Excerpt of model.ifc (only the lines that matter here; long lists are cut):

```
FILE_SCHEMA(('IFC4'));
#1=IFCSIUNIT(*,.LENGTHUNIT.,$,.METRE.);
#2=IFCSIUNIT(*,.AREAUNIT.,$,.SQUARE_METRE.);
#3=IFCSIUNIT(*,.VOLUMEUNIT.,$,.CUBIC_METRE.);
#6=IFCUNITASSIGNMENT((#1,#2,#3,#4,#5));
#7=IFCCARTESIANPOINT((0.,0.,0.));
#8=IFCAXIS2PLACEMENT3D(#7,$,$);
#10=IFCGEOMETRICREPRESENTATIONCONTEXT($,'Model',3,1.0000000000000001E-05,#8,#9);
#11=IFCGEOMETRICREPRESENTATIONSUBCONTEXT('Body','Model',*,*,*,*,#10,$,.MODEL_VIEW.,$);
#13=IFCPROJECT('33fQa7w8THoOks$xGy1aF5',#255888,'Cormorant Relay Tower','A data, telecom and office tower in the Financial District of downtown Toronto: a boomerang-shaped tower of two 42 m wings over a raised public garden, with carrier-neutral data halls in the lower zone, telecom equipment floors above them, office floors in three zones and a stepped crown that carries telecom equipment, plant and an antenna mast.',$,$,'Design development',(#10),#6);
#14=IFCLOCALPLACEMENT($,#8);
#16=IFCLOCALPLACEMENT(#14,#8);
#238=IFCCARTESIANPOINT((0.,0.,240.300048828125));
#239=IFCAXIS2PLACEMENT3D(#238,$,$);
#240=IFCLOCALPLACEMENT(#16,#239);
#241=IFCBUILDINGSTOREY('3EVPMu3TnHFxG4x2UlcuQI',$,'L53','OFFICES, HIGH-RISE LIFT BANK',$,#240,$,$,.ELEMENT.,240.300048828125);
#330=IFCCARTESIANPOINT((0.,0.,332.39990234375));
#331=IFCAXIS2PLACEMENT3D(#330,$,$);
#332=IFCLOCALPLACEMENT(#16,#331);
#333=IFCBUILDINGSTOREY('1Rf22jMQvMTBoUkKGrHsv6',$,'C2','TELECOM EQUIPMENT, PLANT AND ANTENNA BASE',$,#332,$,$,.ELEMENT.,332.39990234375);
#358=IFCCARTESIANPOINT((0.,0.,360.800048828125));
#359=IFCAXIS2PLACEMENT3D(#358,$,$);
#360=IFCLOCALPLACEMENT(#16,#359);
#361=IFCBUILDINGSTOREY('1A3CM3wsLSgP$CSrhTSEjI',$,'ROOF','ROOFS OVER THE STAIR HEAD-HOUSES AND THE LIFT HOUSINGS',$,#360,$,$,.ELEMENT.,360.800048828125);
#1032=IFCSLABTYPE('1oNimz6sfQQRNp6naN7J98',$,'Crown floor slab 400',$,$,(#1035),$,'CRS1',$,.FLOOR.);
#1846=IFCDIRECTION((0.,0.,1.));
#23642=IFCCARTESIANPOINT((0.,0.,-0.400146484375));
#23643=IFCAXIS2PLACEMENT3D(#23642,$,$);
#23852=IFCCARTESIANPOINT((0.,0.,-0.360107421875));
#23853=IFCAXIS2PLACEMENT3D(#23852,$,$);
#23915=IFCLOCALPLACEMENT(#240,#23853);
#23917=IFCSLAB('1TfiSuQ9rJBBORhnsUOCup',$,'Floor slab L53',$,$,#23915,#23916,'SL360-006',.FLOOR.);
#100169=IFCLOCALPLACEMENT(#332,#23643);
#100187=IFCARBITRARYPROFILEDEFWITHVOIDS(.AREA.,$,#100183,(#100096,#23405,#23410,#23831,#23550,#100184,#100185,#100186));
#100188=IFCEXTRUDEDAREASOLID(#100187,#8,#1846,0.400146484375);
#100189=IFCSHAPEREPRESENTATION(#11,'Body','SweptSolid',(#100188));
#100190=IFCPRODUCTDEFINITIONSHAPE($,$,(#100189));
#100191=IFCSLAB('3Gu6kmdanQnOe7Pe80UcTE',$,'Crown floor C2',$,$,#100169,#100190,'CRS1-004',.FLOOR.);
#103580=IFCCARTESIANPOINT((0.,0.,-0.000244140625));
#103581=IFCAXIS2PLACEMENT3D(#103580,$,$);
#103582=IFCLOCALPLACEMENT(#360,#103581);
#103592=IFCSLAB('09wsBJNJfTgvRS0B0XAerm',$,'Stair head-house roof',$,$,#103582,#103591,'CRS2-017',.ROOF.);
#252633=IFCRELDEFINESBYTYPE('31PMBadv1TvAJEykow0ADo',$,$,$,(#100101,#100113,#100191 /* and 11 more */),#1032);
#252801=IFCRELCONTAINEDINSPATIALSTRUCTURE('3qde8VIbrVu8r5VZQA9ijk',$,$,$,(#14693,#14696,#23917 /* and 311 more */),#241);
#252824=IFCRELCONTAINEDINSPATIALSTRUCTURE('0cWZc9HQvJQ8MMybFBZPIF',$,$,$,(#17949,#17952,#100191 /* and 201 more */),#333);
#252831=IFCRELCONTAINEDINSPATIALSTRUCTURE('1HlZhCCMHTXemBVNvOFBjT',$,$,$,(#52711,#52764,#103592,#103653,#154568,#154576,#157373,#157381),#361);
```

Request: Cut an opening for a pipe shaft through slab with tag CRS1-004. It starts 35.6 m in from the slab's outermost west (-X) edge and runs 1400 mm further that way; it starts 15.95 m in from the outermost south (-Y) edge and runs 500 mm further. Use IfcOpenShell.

```python
import numpy as np
import ifcopenshell
import ifcopenshell.api.feature
import ifcopenshell.api.geometry
import ifcopenshell.api.root
import ifcopenshell.geom
import ifcopenshell.util.placement
import ifcopenshell.util.representation
import ifcopenshell.util.shape
import ifcopenshell.util.unit

model = ifcopenshell.open("model.ifc")
unit_scale = ifcopenshell.util.unit.calculate_unit_scale(model)
settings = ifcopenshell.geom.settings()


def volume(element):
    """Net volume in cubic metres, openings subtracted."""
    shape = ifcopenshell.geom.create_shape(settings, element)
    return ifcopenshell.util.shape.get_volume(shape.geometry)


slab = model.by_id(100191)
before = volume(slab)

# Extent in the slab's own axes, in metres. The edges named are its -X and -Y sides.
slab_shape = ifcopenshell.geom.create_shape(settings, slab)
vertices = ifcopenshell.util.shape.get_vertices(slab_shape.geometry)
x_min, y_min, bottom = vertices.min(axis=0)
top = vertices[:, 2].max()

opening = ifcopenshell.api.root.create_entity(model, ifc_class="IfcOpeningElement", name="Pipe shaft opening", predefined_type="OPENING")
context = ifcopenshell.util.representation.get_context(model, "Model", "Body", "MODEL_VIEW")
width, depth = 1.4, 0.5
outline = [(0.0, 0.0), (width, 0.0), (width, depth), (0.0, depth), (0.0, 0.0)]
# Overshoot both faces by 50 mm so the cut is clean.
shape = ifcopenshell.api.geometry.add_slab_representation(
    model, context=context, depth=top - bottom + 0.1, polyline=outline
)
ifcopenshell.api.geometry.assign_representation(model, product=opening, representation=shape)

matrix = ifcopenshell.util.placement.get_local_placement(slab.ObjectPlacement)
matrix[:, 3] = matrix @ np.append(np.array([x_min + 35.6, y_min + 15.95, bottom - 0.05]) / unit_scale, 1.0)
ifcopenshell.api.geometry.edit_object_placement(model, product=opening, matrix=matrix, is_si=False)
ifcopenshell.api.feature.add_feature(model, feature=opening, element=slab)

after = volume(slab)

print(f"slab volume {before:.3f} -> {after:.3f} m3")

model.write("model-out.ifc")
```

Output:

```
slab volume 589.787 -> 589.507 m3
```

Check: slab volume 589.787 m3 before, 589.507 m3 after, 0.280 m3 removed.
